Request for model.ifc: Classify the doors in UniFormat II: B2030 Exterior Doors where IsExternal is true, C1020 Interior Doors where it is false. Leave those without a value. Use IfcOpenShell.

First a look at what the model holds.

```python
import ifcopenshell
import ifcopenshell.util.element

model = ifcopenshell.open("model.ifc")
print(model.schema)
print("classifications:", [c.Name for c in model.by_type("IfcClassification")])
values = [ifcopenshell.util.element.get_pset(e, "Pset_DoorCommon", "IsExternal") for e in model.by_type("IfcDoor")]
for value in (True, False, None):
    print("IsExternal", value, values.count(value))
```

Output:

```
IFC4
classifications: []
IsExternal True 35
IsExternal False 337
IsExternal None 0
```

```python
import ifcopenshell
import ifcopenshell.api.classification
import ifcopenshell.util.element

model = ifcopenshell.open("model.ifc")

system = ifcopenshell.api.classification.add_classification(model, classification="UniFormat II")

doors = model.by_type("IfcDoor")
external = {e: ifcopenshell.util.element.get_pset(e, "Pset_DoorCommon", "IsExternal") for e in doors}
for flag, code, name in ((True, "B2030", "Exterior Doors"), (False, "C1020", "Interior Doors")):
    products = [e for e in doors if external[e] is flag]
    ifcopenshell.api.classification.add_reference(
        model, products=products, classification=system, identification=code, name=name
    )
    print(code, len(products))

model.write("model_rev.ifc")
```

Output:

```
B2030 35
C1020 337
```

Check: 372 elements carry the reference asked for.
